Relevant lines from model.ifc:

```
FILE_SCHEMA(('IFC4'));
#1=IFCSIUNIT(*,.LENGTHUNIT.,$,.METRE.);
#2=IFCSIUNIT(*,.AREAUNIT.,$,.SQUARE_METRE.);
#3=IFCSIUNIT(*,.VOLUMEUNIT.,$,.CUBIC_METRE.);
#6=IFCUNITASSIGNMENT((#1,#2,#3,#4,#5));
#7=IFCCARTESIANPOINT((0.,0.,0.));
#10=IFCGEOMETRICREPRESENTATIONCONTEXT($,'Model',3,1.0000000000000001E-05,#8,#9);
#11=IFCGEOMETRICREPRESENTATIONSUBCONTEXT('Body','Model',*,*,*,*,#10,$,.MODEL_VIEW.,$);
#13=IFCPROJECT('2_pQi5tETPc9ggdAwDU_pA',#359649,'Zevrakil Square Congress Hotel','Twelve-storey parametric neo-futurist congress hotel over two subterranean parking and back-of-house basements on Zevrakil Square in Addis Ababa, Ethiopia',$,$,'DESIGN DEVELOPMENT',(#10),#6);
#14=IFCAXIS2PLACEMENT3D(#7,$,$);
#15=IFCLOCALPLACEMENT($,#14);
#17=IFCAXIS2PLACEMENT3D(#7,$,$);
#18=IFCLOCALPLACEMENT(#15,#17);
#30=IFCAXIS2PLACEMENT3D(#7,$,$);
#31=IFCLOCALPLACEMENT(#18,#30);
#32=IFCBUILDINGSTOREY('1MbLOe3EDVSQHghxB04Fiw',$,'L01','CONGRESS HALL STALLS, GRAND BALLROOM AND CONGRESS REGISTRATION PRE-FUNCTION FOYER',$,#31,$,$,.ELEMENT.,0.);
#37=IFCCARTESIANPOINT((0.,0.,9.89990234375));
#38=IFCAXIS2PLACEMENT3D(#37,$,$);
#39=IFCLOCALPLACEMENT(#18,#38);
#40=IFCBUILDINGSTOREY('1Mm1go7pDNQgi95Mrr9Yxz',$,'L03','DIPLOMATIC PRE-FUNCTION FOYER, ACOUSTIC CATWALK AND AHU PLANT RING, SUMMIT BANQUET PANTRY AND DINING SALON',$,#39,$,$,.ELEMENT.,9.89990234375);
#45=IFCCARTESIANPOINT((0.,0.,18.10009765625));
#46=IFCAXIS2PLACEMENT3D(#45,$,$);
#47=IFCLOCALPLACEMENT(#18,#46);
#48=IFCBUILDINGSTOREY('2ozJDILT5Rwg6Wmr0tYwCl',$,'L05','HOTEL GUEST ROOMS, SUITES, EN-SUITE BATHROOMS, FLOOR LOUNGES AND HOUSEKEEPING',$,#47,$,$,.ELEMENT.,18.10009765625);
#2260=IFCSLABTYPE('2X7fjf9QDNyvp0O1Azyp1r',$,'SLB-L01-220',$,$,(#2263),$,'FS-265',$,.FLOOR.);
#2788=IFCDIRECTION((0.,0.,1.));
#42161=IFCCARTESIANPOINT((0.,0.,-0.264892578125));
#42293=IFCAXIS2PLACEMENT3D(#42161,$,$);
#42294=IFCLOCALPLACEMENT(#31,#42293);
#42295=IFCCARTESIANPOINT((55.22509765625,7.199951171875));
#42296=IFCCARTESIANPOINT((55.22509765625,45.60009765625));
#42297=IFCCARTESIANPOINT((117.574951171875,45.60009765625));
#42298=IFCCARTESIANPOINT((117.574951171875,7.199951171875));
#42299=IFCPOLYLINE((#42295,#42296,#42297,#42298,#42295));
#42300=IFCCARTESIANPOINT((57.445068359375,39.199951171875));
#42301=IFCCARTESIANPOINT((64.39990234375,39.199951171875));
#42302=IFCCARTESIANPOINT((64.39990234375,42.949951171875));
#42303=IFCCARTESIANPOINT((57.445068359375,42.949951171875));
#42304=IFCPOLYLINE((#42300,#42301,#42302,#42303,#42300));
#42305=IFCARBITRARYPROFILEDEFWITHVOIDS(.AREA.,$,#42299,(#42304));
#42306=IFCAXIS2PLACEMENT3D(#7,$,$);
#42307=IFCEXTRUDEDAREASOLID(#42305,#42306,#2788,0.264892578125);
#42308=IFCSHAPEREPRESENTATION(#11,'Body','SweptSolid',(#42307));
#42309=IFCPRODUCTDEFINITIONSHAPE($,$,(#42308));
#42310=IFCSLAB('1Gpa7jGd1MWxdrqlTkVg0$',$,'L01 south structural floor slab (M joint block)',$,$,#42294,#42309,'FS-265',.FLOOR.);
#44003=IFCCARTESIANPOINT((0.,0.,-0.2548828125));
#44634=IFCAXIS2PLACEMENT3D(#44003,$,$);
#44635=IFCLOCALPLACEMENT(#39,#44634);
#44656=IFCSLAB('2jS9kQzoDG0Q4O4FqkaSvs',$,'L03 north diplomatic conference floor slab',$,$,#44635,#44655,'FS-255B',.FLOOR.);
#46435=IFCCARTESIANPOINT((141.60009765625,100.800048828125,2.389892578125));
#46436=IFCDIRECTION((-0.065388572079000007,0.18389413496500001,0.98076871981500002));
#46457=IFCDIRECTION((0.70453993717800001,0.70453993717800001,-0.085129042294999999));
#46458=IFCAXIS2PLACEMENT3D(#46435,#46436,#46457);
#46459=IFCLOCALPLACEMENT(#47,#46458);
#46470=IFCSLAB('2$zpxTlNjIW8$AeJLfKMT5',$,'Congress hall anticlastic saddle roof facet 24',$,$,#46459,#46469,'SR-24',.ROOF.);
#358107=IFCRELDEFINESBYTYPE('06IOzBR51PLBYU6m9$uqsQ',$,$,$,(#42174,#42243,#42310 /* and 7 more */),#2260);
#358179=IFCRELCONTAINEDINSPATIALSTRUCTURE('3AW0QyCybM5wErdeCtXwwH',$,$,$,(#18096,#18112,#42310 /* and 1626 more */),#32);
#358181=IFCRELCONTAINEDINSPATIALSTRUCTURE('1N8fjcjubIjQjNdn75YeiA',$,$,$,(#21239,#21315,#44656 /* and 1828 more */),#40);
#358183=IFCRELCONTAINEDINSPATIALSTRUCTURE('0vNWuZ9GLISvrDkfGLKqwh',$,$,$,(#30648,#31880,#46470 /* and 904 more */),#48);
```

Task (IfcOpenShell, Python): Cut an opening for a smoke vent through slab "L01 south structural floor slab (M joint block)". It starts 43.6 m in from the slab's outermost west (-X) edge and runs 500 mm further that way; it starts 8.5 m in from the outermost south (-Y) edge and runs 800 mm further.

```python
import numpy as np
import ifcopenshell
import ifcopenshell.api.feature
import ifcopenshell.api.geometry
import ifcopenshell.api.root
import ifcopenshell.geom
import ifcopenshell.util.placement
import ifcopenshell.util.representation
import ifcopenshell.util.shape
import ifcopenshell.util.unit

model = ifcopenshell.open("model.ifc")
unit_scale = ifcopenshell.util.unit.calculate_unit_scale(model)
settings = ifcopenshell.geom.settings()


def volume(element):
    """Net volume in cubic metres, openings subtracted."""
    shape = ifcopenshell.geom.create_shape(settings, element)
    return ifcopenshell.util.shape.get_volume(shape.geometry)


slab = model.by_id(42310)
before = volume(slab)

# Extent in the slab's own axes, in metres. The edges named are its -X and -Y sides.
slab_shape = ifcopenshell.geom.create_shape(settings, slab)
vertices = ifcopenshell.util.shape.get_vertices(slab_shape.geometry)
x_min, y_min, bottom = vertices.min(axis=0)
top = vertices[:, 2].max()

opening = ifcopenshell.api.root.create_entity(model, ifc_class="IfcOpeningElement", name="Smoke vent opening", predefined_type="OPENING")
context = ifcopenshell.util.representation.get_context(model, "Model", "Body", "MODEL_VIEW")
width, depth = 0.5, 0.8
outline = [(0.0, 0.0), (width, 0.0), (width, depth), (0.0, depth), (0.0, 0.0)]
# Overshoot both faces by 50 mm so the cut is clean.
shape = ifcopenshell.api.geometry.add_slab_representation(
    model, context=context, depth=top - bottom + 0.1, polyline=outline
)
ifcopenshell.api.geometry.assign_representation(model, product=opening, representation=shape)

matrix = ifcopenshell.util.placement.get_local_placement(slab.ObjectPlacement)
matrix[:, 3] = matrix @ np.append(np.array([x_min + 43.6, y_min + 8.5, bottom - 0.05]) / unit_scale, 1.0)
ifcopenshell.api.geometry.edit_object_placement(model, product=opening, matrix=matrix, is_si=False)
ifcopenshell.api.feature.add_feature(model, feature=opening, element=slab)

after = volume(slab)

print(f"slab volume {before:.3f} -> {after:.3f} m3")

model.write("model_v2.ifc")
```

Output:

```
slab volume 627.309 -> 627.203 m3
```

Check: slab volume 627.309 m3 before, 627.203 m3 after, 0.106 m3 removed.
